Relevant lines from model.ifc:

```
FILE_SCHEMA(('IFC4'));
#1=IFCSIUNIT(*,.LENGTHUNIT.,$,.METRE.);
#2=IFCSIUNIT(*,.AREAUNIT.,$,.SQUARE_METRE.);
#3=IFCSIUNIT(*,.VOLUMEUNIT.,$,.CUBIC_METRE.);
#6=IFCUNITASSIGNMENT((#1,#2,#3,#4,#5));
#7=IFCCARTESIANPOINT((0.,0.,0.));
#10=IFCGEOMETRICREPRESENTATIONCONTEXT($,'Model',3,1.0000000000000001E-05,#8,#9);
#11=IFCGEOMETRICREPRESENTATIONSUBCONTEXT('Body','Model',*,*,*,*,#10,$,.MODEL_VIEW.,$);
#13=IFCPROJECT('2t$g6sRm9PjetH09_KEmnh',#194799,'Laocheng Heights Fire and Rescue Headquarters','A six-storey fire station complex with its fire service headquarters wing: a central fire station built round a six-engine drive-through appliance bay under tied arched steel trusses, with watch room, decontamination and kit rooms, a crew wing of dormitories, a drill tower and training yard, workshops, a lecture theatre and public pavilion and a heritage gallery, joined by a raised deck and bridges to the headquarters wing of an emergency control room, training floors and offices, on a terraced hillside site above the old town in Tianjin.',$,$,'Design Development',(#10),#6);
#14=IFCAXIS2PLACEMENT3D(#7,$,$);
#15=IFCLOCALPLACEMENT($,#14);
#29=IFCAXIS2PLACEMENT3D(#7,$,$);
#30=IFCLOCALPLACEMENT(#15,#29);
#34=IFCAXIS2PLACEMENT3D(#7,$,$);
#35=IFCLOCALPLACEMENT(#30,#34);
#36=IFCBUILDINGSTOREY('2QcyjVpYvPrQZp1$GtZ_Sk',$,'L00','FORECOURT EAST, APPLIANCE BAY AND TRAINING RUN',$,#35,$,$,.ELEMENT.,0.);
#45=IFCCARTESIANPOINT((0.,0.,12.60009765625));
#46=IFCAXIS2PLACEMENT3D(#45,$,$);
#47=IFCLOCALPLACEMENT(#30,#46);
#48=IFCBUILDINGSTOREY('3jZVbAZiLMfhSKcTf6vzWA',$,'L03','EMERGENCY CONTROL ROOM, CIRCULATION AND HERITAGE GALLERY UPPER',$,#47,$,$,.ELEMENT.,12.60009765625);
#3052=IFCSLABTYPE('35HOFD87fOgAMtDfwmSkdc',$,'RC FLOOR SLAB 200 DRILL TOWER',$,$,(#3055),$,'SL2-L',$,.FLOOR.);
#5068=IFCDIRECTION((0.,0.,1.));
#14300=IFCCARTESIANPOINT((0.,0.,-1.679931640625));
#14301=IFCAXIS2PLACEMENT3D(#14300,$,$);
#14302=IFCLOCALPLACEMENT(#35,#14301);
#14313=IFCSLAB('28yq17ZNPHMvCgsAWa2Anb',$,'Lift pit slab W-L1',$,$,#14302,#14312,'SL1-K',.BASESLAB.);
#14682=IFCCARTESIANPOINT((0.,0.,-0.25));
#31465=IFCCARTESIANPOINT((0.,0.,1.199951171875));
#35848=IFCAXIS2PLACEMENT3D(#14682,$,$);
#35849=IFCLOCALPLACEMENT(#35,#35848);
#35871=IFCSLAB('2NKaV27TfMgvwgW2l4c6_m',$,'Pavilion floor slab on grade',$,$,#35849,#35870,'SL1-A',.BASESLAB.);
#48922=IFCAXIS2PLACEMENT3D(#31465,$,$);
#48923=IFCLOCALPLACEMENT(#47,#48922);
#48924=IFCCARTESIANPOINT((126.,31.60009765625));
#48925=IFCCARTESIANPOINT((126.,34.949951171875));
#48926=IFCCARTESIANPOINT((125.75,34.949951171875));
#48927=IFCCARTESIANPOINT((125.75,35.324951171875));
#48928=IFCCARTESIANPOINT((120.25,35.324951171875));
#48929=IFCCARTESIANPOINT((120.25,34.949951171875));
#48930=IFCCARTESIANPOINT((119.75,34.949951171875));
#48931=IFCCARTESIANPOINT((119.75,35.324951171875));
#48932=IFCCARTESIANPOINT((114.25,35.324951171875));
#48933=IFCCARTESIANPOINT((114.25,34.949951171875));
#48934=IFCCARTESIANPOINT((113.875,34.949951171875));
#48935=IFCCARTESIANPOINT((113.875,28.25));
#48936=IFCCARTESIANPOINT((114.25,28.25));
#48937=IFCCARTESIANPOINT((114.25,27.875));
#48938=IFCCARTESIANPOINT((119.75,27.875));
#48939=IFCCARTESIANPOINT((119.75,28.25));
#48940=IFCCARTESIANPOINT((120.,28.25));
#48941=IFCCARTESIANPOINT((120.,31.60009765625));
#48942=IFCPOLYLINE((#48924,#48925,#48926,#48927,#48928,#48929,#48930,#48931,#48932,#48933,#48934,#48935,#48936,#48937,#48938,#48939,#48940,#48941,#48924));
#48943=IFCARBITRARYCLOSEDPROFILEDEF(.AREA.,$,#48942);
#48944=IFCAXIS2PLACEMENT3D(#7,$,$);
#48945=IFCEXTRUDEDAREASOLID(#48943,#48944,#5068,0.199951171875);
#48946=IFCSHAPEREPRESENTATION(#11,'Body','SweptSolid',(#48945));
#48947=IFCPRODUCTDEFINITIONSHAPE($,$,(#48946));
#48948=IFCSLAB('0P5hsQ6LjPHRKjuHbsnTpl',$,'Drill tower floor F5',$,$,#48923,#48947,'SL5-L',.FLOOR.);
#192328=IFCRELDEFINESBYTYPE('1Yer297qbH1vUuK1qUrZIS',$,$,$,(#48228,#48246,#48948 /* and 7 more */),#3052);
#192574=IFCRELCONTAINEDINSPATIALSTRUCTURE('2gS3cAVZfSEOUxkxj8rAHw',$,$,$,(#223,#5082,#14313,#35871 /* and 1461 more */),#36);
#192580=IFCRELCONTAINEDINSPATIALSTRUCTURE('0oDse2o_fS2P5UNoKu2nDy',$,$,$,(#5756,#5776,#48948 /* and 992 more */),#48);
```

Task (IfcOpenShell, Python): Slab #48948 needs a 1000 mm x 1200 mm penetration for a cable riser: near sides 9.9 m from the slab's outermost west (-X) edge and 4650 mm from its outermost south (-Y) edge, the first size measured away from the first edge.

```python
import numpy as np
import ifcopenshell
import ifcopenshell.api.feature
import ifcopenshell.api.geometry
import ifcopenshell.api.root
import ifcopenshell.geom
import ifcopenshell.util.placement
import ifcopenshell.util.representation
import ifcopenshell.util.shape
import ifcopenshell.util.unit

model = ifcopenshell.open("model.ifc")
unit_scale = ifcopenshell.util.unit.calculate_unit_scale(model)
settings = ifcopenshell.geom.settings()


def volume(element):
    """Net volume in cubic metres, openings subtracted."""
    shape = ifcopenshell.geom.create_shape(settings, element)
    return ifcopenshell.util.shape.get_volume(shape.geometry)


slab = model.by_guid("0P5hsQ6LjPHRKjuHbsnTpl")
before = volume(slab)

# Extent in the slab's own axes, in metres. The edges named are its -X and -Y sides.
slab_shape = ifcopenshell.geom.create_shape(settings, slab)
vertices = ifcopenshell.util.shape.get_vertices(slab_shape.geometry)
x_min, y_min, bottom = vertices.min(axis=0)
top = vertices[:, 2].max()

opening = ifcopenshell.api.root.create_entity(model, ifc_class="IfcOpeningElement", name="Cable riser opening", predefined_type="OPENING")
context = ifcopenshell.util.representation.get_context(model, "Model", "Body", "MODEL_VIEW")
width, depth = 1, 1.2
outline = [(0.0, 0.0), (width, 0.0), (width, depth), (0.0, depth), (0.0, 0.0)]
# Overshoot both faces by 50 mm so the cut is clean.
shape = ifcopenshell.api.geometry.add_slab_representation(
    model, context=context, depth=top - bottom + 0.1, polyline=outline
)
ifcopenshell.api.geometry.assign_representation(model, product=opening, representation=shape)

matrix = ifcopenshell.util.placement.get_local_placement(slab.ObjectPlacement)
matrix[:, 3] = matrix @ np.append(np.array([x_min + 9.9, y_min + 4.65, bottom - 0.05]) / unit_scale, 1.0)
ifcopenshell.api.geometry.edit_object_placement(model, product=opening, matrix=matrix, is_si=False)
ifcopenshell.api.feature.add_feature(model, feature=opening, element=slab)

after = volume(slab)

print(f"slab volume {before:.3f} -> {after:.3f} m3")

model.write("model_v2.ifc")
```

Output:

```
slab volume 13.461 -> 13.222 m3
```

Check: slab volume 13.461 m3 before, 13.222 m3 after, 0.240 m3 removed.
